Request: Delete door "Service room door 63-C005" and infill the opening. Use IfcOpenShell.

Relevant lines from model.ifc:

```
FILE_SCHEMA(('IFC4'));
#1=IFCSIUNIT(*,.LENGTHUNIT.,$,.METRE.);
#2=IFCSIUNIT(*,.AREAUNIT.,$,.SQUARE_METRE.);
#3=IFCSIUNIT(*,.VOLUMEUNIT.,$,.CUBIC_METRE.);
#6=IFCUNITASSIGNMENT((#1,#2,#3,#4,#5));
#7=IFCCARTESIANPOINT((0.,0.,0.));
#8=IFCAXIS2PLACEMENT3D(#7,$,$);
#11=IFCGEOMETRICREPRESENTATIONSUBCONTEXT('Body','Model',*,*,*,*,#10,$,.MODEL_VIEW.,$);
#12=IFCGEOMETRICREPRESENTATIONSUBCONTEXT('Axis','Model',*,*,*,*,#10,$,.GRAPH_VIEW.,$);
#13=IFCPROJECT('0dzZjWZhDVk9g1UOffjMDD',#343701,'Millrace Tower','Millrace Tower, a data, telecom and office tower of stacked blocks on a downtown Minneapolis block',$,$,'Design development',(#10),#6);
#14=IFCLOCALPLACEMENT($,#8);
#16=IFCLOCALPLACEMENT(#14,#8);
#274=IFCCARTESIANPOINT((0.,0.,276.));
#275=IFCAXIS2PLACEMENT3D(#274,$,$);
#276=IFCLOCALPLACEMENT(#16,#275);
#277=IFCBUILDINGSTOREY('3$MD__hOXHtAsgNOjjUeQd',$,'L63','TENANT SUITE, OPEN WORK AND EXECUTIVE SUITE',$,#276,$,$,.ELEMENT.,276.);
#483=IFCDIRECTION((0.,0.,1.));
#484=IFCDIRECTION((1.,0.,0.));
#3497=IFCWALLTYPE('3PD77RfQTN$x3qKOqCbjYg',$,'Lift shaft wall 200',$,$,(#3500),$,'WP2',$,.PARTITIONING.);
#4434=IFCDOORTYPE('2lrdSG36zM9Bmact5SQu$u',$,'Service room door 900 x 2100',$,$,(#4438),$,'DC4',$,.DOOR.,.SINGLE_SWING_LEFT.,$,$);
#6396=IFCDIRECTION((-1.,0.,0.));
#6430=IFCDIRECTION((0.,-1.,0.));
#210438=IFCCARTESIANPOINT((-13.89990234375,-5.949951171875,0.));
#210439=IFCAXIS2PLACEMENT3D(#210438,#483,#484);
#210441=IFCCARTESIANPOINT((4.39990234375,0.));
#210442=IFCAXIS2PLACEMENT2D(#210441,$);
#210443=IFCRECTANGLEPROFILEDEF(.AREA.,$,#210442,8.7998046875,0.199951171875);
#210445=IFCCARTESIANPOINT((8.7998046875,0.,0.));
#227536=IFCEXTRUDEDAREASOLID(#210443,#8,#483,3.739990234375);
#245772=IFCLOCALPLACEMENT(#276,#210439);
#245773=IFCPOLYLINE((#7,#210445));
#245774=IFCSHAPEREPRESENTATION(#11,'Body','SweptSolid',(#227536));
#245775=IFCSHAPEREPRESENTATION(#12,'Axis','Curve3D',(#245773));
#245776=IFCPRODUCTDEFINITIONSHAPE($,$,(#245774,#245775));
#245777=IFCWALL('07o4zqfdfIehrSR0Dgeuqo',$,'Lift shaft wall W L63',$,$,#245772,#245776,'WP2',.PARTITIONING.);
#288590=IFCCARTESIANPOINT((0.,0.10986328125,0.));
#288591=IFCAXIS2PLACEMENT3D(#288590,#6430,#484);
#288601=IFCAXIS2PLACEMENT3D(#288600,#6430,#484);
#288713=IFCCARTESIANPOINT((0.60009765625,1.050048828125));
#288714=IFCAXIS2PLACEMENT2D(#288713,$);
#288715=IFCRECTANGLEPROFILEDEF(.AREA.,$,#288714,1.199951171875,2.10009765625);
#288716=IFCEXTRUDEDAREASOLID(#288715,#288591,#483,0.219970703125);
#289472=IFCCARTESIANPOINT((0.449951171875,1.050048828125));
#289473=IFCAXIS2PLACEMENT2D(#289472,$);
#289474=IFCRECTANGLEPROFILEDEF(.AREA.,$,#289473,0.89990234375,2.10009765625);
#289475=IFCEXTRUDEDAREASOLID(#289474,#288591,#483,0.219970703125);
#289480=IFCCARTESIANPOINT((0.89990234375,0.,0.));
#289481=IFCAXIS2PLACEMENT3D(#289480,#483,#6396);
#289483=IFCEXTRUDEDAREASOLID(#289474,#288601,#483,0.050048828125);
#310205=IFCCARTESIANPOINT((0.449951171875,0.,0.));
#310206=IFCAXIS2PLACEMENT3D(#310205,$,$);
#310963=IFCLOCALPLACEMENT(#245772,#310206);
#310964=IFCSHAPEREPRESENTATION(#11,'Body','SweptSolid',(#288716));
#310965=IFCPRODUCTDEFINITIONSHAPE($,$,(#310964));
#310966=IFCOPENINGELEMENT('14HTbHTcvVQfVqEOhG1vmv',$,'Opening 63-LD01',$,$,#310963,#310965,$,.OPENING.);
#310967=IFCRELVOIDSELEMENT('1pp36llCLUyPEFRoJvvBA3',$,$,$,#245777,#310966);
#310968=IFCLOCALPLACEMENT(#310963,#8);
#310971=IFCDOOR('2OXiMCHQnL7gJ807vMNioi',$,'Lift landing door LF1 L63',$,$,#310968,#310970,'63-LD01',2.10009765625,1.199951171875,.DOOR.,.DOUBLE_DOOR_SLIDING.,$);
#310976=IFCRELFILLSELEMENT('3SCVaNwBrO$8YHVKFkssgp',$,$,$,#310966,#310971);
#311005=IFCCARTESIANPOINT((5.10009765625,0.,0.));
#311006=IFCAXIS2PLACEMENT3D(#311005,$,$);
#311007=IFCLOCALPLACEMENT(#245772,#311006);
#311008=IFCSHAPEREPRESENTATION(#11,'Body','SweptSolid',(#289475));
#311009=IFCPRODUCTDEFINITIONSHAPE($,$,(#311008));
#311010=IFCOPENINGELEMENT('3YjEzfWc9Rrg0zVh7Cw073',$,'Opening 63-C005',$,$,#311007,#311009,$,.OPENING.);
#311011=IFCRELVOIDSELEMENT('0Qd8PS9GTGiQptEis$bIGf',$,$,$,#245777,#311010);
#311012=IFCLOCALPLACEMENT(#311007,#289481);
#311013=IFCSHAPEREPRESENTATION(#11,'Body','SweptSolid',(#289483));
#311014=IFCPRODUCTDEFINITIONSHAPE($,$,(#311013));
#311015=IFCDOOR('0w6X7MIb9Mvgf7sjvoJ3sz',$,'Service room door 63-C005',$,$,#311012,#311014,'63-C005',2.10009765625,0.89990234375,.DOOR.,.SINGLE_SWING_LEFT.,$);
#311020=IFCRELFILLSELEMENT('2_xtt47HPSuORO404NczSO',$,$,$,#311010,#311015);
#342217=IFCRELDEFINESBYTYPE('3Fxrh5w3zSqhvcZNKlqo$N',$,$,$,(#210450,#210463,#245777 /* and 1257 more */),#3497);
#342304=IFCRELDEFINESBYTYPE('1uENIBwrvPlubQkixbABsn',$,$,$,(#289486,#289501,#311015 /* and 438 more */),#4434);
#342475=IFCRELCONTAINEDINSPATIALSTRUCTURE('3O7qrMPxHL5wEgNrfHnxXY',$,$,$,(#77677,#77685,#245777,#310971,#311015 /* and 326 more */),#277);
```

```python
import ifcopenshell
import ifcopenshell.api.feature
import ifcopenshell.api.root
import ifcopenshell.geom
import ifcopenshell.util.shape

model = ifcopenshell.open("model.ifc")
settings = ifcopenshell.geom.settings()


def volume(element):
    """Net volume in cubic metres, openings subtracted."""
    shape = ifcopenshell.geom.create_shape(settings, element)
    return ifcopenshell.util.shape.get_volume(shape.geometry)


door = model.by_guid("0w6X7MIb9Mvgf7sjvoJ3sz")
opening = door.FillsVoids[0].RelatingOpeningElement
wall = opening.VoidsElements[0].RelatingBuildingElement
before = volume(wall)

ifcopenshell.api.root.remove_product(model, product=door)
ifcopenshell.api.feature.remove_feature(model, feature=opening)

after = volume(wall)

print(f"wall volume {before:.3f} -> {after:.3f} m3")

model.write("model_edited.ifc")
```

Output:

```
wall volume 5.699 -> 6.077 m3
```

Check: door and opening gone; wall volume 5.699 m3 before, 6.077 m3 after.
